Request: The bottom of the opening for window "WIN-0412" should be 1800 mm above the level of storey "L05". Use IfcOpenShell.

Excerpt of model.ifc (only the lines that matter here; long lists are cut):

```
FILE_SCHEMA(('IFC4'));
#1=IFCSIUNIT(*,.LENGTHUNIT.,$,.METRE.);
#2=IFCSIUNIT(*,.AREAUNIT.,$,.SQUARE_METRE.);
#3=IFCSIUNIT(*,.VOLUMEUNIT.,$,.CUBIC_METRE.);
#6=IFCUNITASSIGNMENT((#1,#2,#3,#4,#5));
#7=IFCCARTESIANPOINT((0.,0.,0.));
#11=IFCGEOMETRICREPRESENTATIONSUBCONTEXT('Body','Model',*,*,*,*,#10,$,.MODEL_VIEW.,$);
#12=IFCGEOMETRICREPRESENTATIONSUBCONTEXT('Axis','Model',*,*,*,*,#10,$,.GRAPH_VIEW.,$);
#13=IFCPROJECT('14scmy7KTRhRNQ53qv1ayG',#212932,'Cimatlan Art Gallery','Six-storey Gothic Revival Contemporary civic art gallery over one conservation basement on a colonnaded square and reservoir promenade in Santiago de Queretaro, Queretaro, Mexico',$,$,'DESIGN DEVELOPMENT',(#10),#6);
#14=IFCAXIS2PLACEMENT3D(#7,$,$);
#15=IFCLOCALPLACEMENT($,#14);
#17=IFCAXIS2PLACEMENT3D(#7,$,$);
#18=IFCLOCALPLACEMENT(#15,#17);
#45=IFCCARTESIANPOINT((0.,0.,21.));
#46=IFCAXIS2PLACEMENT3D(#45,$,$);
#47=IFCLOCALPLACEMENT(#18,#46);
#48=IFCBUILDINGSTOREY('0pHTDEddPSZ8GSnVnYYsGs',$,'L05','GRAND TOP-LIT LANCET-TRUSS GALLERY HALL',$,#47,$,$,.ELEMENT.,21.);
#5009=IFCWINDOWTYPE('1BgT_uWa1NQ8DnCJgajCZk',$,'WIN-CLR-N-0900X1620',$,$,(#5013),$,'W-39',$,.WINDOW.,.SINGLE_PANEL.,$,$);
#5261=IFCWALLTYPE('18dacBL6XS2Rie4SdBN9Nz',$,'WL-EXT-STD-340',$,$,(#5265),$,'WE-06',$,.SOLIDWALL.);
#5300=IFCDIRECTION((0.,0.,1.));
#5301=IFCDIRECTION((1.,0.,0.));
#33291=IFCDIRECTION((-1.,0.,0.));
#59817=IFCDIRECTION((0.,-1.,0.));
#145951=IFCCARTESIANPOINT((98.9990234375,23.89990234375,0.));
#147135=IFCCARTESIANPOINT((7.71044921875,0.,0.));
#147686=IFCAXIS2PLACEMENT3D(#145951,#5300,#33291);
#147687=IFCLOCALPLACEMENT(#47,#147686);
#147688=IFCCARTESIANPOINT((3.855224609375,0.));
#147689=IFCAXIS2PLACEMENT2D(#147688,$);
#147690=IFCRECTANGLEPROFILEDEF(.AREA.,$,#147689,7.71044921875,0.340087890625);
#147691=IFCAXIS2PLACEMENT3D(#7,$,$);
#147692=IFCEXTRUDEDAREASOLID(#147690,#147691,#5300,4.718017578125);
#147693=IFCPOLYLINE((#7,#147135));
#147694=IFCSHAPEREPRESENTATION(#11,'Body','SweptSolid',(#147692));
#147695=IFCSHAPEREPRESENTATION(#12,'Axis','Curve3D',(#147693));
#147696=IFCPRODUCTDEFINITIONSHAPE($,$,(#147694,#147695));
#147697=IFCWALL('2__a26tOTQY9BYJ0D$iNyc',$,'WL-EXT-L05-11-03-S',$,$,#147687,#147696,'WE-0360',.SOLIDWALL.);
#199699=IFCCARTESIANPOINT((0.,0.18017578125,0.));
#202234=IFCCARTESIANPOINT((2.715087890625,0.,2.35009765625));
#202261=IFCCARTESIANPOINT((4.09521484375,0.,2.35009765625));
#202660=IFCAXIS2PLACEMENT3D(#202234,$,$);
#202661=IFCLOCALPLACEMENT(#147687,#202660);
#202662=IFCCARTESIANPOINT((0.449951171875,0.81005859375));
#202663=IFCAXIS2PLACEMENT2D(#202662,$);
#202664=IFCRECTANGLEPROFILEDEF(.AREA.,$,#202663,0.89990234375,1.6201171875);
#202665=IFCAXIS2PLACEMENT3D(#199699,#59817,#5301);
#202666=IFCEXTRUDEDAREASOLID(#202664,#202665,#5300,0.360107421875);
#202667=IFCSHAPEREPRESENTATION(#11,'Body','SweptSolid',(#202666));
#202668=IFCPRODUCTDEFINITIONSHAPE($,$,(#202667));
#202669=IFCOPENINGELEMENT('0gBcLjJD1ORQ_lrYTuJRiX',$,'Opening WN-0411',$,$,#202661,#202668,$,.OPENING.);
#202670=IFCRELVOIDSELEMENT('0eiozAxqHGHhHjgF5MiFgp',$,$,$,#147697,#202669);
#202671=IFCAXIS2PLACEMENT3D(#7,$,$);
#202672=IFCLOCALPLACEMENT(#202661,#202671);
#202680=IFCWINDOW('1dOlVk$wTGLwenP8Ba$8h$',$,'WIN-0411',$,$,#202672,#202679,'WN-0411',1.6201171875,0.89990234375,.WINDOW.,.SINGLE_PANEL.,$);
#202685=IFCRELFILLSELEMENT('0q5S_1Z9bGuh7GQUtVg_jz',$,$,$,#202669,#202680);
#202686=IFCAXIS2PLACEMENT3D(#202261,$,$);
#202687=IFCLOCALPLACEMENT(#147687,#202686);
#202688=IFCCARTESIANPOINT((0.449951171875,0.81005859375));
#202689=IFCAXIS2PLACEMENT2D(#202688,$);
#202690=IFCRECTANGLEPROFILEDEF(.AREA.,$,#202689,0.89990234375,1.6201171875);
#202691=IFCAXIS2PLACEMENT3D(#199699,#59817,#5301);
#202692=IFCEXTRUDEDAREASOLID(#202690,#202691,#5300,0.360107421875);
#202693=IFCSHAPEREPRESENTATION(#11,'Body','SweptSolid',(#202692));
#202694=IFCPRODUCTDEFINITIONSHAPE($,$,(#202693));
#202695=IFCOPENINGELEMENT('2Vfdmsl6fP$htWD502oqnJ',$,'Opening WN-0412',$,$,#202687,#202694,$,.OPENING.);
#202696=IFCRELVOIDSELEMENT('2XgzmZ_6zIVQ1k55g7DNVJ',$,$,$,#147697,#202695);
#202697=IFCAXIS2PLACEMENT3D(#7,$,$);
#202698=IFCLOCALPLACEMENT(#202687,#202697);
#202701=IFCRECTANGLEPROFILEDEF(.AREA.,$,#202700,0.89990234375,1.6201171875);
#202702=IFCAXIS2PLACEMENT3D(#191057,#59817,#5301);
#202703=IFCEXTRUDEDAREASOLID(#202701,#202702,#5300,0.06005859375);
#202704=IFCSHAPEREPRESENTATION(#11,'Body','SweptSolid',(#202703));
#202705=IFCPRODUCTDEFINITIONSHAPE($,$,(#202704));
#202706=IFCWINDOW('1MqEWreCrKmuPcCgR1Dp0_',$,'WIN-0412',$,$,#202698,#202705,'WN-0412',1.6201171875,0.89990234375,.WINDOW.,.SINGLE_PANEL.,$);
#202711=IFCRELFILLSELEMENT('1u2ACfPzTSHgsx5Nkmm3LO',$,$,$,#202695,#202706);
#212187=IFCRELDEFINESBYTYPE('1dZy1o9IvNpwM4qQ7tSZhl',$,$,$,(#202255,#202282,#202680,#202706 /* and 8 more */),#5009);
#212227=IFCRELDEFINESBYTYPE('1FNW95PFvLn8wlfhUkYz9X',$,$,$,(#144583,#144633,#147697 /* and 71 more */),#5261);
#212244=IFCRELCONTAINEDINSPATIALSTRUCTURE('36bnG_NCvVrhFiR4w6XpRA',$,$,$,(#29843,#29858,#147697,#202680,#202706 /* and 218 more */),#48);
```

```python
import numpy as np
import ifcopenshell
import ifcopenshell.api.geometry
import ifcopenshell.geom
import ifcopenshell.util.element
import ifcopenshell.util.placement
import ifcopenshell.util.shape
import ifcopenshell.util.unit

model = ifcopenshell.open("model.ifc")
unit_scale = ifcopenshell.util.unit.calculate_unit_scale(model)

window = model.by_id(202706)
opening = window.FillsVoids[0].RelatingOpeningElement
storey = ifcopenshell.util.element.get_container(window, ifc_class="IfcBuildingStorey")
level = ifcopenshell.util.placement.get_local_placement(storey.ObjectPlacement)[2, 3]

# The opening's origin need not be at the sill, so measure its lowest point.
shape = ifcopenshell.geom.create_shape(ifcopenshell.geom.settings(), opening)
bottom = ifcopenshell.util.shape.get_shape_bottom_elevation(shape, shape.geometry) / unit_scale
dz = level + 1.8 / unit_scale - bottom

shift = np.array([0.0, 0.0, dz])
# The window is placed relative to its opening, so it follows when the opening moves.
matrix = ifcopenshell.util.placement.get_local_placement(opening.ObjectPlacement)
matrix[:3, 3] += shift
ifcopenshell.api.geometry.edit_object_placement(
    model, product=opening, matrix=matrix, is_si=False, should_transform_children=True
)

print(f"moved by {dz * unit_scale:+.3f} m")

model.write("model_rev.ifc")
```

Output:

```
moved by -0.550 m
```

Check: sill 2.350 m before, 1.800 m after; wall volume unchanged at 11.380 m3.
